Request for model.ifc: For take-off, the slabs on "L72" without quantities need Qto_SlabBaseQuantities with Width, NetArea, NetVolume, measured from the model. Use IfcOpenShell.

First a look at what the model holds.

```python
import ifcopenshell
import ifcopenshell.util.element
import ifcopenshell.util.unit

model = ifcopenshell.open("model.ifc")
print(model.schema)
for unit_type in ("LENGTHUNIT", "AREAUNIT", "VOLUMEUNIT"):
    print(unit_type, ifcopenshell.util.unit.calculate_unit_scale(model, unit_type))
storey = next(s for s in model.by_type("IfcBuildingStorey") if s.Name == "L72")
slabs = [e for e in ifcopenshell.util.element.get_decomposition(storey) if e.is_a("IfcSlab")]
for e in sorted(slabs, key=lambda e: e.id()):
    print(e.id(), e.is_a(), e.Name, list(ifcopenshell.util.element.get_psets(e, qtos_only=True)), sep=" | ")
```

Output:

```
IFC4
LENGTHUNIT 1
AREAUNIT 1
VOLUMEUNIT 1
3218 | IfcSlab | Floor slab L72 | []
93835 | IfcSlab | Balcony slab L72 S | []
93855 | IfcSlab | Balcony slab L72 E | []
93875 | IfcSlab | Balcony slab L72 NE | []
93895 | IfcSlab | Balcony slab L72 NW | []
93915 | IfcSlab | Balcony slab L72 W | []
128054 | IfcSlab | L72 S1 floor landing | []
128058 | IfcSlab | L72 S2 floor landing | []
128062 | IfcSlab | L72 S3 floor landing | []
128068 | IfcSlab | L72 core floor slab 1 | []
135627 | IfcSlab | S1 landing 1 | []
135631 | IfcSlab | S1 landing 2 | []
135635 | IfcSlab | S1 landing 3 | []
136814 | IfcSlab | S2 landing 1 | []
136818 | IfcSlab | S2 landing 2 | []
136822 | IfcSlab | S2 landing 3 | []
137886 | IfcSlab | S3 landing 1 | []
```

```python
import ifcopenshell
import ifcopenshell.api.pset
import ifcopenshell.geom
import ifcopenshell.util.element
import ifcopenshell.util.shape
import ifcopenshell.util.unit

model = ifcopenshell.open("model.ifc")
unit_scale = ifcopenshell.util.unit.calculate_unit_scale(model)
area_scale = ifcopenshell.util.unit.calculate_unit_scale(model, "AREAUNIT")
volume_scale = ifcopenshell.util.unit.calculate_unit_scale(model, "VOLUMEUNIT")
settings = ifcopenshell.geom.settings()

storey = next(s for s in model.by_type("IfcBuildingStorey") if s.Name == "L72")
slabs = [e for e in ifcopenshell.util.element.get_decomposition(storey) if e.is_a("IfcSlab")]

for e in sorted(slabs, key=lambda e: e.id()):
    if ifcopenshell.util.element.get_psets(e, qtos_only=True, should_inherit=False):
        continue
    # Geometry comes back in metres, in the element's own axes.
    shape = ifcopenshell.geom.create_shape(settings, e)
    values = {
        "Width": ifcopenshell.util.shape.get_z(shape.geometry) / unit_scale,
        "NetArea": ifcopenshell.util.shape.get_footprint_area(shape.geometry) / area_scale,
        "NetVolume": ifcopenshell.util.shape.get_volume(shape.geometry) / volume_scale,
    }
    qto = ifcopenshell.api.pset.add_qto(model, product=e, name="Qto_SlabBaseQuantities")
    ifcopenshell.api.pset.edit_qto(model, qto=qto, properties=values)
    print(e.id(), {k: round(v, 3) for k, v in values.items()})

model.write("model_rev.ifc")
```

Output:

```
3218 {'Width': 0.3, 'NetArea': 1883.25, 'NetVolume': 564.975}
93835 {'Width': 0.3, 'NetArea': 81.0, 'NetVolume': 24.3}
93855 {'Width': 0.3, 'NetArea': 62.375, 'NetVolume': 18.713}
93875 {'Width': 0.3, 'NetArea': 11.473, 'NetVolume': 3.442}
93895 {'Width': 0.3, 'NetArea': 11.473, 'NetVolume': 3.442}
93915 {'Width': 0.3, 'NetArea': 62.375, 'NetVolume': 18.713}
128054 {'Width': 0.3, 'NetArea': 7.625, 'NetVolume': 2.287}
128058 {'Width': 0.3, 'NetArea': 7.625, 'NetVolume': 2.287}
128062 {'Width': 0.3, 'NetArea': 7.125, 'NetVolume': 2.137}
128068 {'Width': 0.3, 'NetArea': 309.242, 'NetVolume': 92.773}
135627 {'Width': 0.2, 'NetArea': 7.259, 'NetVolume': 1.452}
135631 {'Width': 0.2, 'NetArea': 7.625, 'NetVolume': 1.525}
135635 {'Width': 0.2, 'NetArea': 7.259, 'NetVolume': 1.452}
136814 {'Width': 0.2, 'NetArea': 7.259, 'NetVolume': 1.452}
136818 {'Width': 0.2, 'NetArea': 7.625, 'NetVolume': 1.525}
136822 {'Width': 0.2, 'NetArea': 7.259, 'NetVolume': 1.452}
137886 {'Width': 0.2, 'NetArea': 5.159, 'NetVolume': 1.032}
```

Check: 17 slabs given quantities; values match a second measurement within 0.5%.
